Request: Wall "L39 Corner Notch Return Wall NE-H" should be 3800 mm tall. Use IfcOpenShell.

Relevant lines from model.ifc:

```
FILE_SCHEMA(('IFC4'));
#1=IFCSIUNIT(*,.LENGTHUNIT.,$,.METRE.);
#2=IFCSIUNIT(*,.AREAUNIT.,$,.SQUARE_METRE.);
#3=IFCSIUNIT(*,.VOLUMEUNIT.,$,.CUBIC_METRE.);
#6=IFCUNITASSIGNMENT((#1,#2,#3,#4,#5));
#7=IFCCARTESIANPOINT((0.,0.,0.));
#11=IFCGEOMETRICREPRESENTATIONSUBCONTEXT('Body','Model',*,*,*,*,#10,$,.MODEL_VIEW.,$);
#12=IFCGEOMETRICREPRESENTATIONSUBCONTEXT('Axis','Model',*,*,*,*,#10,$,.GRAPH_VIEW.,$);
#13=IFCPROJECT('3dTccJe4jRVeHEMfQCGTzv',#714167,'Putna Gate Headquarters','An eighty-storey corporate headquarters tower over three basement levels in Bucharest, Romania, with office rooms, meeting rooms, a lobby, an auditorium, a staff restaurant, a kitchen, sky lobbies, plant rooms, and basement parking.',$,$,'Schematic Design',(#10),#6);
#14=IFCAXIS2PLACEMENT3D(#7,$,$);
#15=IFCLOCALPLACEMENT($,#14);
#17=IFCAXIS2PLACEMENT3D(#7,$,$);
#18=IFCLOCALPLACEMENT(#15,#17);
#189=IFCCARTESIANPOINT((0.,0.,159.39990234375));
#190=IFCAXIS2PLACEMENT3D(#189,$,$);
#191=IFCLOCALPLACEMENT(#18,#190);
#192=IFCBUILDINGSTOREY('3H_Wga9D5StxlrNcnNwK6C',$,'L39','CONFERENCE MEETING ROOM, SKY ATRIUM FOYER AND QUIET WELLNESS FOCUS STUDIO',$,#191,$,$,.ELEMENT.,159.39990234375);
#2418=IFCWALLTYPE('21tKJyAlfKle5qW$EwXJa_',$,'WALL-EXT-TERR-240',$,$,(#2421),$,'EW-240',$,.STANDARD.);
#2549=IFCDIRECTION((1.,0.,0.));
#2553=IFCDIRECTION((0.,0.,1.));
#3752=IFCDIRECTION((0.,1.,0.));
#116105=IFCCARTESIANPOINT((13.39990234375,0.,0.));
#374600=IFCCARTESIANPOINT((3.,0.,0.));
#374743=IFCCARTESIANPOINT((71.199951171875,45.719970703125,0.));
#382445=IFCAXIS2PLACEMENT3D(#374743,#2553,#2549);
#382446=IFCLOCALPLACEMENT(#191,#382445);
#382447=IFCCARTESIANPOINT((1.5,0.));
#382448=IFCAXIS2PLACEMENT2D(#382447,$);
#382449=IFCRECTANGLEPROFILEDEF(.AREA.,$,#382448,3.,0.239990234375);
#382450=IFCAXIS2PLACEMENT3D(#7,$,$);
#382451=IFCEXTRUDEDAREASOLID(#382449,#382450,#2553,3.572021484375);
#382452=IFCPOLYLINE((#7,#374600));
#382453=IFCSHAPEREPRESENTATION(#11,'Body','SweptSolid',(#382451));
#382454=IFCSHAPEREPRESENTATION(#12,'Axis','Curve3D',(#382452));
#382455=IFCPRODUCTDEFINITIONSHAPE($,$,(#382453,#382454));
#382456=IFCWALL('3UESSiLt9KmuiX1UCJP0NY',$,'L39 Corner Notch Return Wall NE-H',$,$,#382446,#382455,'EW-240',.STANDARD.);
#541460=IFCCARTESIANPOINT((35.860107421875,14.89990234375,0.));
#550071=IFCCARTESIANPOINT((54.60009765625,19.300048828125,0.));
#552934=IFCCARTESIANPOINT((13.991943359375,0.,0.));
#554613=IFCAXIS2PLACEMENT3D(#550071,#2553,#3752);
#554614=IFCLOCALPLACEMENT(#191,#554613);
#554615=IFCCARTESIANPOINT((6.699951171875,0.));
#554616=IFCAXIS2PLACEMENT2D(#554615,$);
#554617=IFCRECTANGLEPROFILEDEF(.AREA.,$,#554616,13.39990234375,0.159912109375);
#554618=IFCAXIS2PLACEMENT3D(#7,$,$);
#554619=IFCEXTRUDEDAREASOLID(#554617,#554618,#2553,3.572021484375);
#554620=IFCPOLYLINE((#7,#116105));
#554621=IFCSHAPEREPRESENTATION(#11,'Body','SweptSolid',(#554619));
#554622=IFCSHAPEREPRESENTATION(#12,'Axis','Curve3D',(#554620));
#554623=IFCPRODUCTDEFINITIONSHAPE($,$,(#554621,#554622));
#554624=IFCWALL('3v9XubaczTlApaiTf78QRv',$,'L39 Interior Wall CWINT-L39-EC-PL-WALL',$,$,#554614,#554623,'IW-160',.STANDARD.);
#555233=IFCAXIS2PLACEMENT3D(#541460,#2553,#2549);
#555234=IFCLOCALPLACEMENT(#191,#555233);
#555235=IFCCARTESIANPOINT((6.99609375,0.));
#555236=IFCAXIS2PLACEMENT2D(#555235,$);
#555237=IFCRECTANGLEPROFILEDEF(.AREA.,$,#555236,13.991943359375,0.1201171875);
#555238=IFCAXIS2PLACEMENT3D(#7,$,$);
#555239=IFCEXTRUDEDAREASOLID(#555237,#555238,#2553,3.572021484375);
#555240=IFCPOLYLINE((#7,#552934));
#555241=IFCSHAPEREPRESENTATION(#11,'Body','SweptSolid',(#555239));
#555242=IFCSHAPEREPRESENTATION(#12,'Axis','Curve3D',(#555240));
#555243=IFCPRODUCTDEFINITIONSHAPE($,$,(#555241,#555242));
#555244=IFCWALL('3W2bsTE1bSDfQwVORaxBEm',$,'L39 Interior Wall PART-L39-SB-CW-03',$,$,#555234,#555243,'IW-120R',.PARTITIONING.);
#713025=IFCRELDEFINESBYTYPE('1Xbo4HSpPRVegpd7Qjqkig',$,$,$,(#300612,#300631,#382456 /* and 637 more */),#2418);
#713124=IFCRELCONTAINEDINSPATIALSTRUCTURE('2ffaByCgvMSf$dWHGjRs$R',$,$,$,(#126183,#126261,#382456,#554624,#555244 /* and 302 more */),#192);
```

```python
import ifcopenshell
import ifcopenshell.geom
import ifcopenshell.util.representation
import ifcopenshell.util.shape

model = ifcopenshell.open("model.ifc")
settings = ifcopenshell.geom.settings()


def volume(element):
    """Net volume in cubic metres, openings subtracted."""
    shape = ifcopenshell.geom.create_shape(settings, element)
    return ifcopenshell.util.shape.get_volume(shape.geometry)


wall = model.by_guid("3UESSiLt9KmuiX1UCJP0NY")
before = volume(wall)

body = ifcopenshell.util.representation.get_representation(wall, "Model", "Body")
solid = body.Items[0]
old_height = solid.Depth
solid.Depth = 3.8
after = volume(wall)

print(f"height {old_height:g} -> {solid.Depth:g}, volume {before:.3f} -> {after:.3f} m3")

model.write("model_edited.ifc")
```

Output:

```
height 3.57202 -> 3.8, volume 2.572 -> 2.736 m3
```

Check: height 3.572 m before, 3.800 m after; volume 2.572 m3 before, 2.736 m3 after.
